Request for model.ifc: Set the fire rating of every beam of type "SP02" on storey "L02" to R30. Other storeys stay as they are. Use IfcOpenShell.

First a look at what the model holds.

```python
import ifcopenshell
import ifcopenshell.util.element

model = ifcopenshell.open("model.ifc")
print(model.schema)
storey = next(s for s in model.by_type("IfcBuildingStorey") if s.Name == "L02")
beams = [e for e in ifcopenshell.util.element.get_decomposition(storey) if e.is_a("IfcBeam")]
seen = {}
for e in beams:
    element_type = ifcopenshell.util.element.get_type(e)
    key = (element_type.Name if element_type != e and element_type else None, ifcopenshell.util.element.get_pset(e, "Pset_BeamCommon", "FireRating"))
    seen[key] = seen.get(key, 0) + 1
for (name, value), count in sorted(seen.items(), key=str):
    print(count, "x", name, "|", value)
```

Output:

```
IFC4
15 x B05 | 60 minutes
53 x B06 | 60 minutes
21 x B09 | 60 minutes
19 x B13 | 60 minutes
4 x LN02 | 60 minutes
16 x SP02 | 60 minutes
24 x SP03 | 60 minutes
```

```python
import ifcopenshell
import ifcopenshell.api.pset
import ifcopenshell.util.element

model = ifcopenshell.open("model.ifc")

storey = next(s for s in model.by_type("IfcBuildingStorey") if s.Name == "L02")
beams = [e for e in ifcopenshell.util.element.get_decomposition(storey) if e.is_a("IfcBeam")]

count = 0
for e in beams:
    element_type = ifcopenshell.util.element.get_type(e)
    if element_type in (None, e) or element_type.Name != "SP02":
        continue
    # add_pset returns the element's existing set when there is one.
    pset = ifcopenshell.api.pset.add_pset(model, product=e, name="Pset_BeamCommon")
    ifcopenshell.api.pset.edit_pset(model, pset=pset, properties={"FireRating": "R30"})
    count += 1

print(count, "beams updated")

model.write("model_rev.ifc")
```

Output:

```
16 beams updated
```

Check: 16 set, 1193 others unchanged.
